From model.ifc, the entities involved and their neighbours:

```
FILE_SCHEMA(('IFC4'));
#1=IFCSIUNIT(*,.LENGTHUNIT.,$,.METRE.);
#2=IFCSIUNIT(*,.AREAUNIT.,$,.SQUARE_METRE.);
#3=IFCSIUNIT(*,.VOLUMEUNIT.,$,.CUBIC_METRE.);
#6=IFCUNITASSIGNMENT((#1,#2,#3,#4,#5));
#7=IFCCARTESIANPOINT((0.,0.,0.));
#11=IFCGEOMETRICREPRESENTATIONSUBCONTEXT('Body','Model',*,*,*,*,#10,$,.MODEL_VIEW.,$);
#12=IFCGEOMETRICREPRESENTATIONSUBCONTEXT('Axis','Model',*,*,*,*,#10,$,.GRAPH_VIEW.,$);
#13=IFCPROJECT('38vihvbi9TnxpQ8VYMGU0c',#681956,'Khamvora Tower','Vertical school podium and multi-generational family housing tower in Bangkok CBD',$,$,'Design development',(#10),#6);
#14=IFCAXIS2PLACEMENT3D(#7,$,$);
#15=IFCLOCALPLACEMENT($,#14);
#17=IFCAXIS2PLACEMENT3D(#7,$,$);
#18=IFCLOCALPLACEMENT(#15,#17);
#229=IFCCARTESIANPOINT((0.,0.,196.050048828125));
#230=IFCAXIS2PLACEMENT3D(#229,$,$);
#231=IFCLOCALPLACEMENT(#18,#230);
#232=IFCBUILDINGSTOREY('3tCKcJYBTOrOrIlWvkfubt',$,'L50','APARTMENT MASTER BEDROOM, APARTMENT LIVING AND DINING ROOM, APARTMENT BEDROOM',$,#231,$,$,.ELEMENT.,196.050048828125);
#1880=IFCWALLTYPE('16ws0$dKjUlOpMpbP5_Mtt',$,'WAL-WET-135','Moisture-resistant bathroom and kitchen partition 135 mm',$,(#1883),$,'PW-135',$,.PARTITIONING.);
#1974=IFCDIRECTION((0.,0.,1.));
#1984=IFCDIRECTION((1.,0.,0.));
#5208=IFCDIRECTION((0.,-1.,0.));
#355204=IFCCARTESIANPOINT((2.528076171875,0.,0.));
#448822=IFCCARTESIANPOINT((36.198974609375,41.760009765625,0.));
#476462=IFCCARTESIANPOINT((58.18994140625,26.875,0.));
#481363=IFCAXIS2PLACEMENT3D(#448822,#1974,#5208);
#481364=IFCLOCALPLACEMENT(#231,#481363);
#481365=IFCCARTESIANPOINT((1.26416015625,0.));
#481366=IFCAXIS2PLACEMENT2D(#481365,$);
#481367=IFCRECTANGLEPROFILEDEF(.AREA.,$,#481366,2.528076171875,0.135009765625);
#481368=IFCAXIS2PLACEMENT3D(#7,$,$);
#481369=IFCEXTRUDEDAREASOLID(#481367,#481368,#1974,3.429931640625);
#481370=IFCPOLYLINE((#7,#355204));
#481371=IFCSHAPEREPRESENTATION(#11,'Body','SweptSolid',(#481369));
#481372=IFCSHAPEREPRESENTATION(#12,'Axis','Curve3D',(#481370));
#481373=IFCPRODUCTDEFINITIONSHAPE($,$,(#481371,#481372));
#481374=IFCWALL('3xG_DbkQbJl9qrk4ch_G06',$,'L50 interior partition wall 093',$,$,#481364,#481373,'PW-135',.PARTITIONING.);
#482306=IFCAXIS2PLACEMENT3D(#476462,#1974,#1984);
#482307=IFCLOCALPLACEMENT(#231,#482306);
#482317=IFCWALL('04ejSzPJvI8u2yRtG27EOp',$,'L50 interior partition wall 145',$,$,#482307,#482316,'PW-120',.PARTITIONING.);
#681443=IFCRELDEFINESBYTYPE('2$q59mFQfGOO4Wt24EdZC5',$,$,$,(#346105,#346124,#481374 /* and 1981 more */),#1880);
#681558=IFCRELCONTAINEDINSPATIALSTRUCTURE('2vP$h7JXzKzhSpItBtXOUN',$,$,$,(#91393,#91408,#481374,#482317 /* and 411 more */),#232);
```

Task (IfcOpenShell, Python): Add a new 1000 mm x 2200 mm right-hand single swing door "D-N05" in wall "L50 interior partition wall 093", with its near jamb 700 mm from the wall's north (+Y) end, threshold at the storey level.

```python
import numpy as np
import ifcopenshell
import ifcopenshell.api.feature
import ifcopenshell.api.geometry
import ifcopenshell.api.root
import ifcopenshell.api.spatial
import ifcopenshell.geom
import ifcopenshell.util.element
import ifcopenshell.util.placement
import ifcopenshell.util.representation
import ifcopenshell.util.shape
import ifcopenshell.util.unit

model = ifcopenshell.open("model.ifc")
unit_scale = ifcopenshell.util.unit.calculate_unit_scale(model)
settings = ifcopenshell.geom.settings()


def volume(element):
    """Net volume in cubic metres, openings subtracted."""
    shape = ifcopenshell.geom.create_shape(settings, element)
    return ifcopenshell.util.shape.get_volume(shape.geometry)


wall = model.by_id(481374)
storey = ifcopenshell.util.element.get_container(wall, ifc_class="IfcBuildingStorey")
context = ifcopenshell.util.representation.get_context(model, "Model", "Body", "MODEL_VIEW")
before = volume(wall)

width, height, from_end, sill = 1, 2.2, 0.7, 0.0  # metres

# The wall runs along its own X axis, and the end named is its -X end.
wall_shape = ifcopenshell.geom.create_shape(settings, wall)
x, y, z = ifcopenshell.util.shape.get_vertices(wall_shape.geometry).T
start = x.min() + from_end
face, thickness = float(y.min()), float(y.max() - y.min())
wall_matrix = ifcopenshell.util.placement.get_local_placement(wall.ObjectPlacement)
level = ifcopenshell.util.placement.get_local_placement(storey.ObjectPlacement)[2, 3]


def in_wall(x, y):
    """Placement at x, y metres in the wall's axes, at sill height."""
    matrix = wall_matrix.copy()
    matrix[:, 3] = wall_matrix @ np.array([x / unit_scale, y / unit_scale, 0.0, 1.0])
    matrix[2, 3] = level + sill / unit_scale
    return matrix


# Opening: a box that overshoots both wall faces by 50 mm.
opening = ifcopenshell.api.root.create_entity(model, ifc_class="IfcOpeningElement", predefined_type="OPENING")
box = ifcopenshell.api.geometry.add_wall_representation(
    model, context=context, length=width, height=height, thickness=thickness + 0.1
)
ifcopenshell.api.geometry.assign_representation(model, product=opening, representation=box)
ifcopenshell.api.geometry.edit_object_placement(model, product=opening, matrix=in_wall(start, face - 0.05), is_si=False)
ifcopenshell.api.feature.add_feature(model, feature=opening, element=wall)

door = ifcopenshell.api.root.create_entity(model, ifc_class="IfcDoor", name="D-N05", predefined_type="DOOR")
door.OverallWidth, door.OverallHeight = width / unit_scale, height / unit_scale
door.OperationType = "SINGLE_SWING_RIGHT"
body = ifcopenshell.api.geometry.add_door_representation(
    model,
    context=context,
    overall_width=door.OverallWidth,
    overall_height=door.OverallHeight,
    operation_type="SINGLE_SWING_RIGHT",
    lining_properties={"LiningDepth": thickness / unit_scale, "ThresholdDepth": thickness / unit_scale},
)
ifcopenshell.api.geometry.assign_representation(model, product=door, representation=body)
ifcopenshell.api.spatial.assign_container(model, products=[door], relating_structure=storey)
ifcopenshell.api.feature.add_filling(model, opening=opening, element=door)

# The lining spans the wall, so the door starts at the wall face.
ifcopenshell.api.geometry.edit_object_placement(model, product=door, matrix=in_wall(start, face), is_si=False)

after = volume(wall)

print(f"wall volume {before:.3f} -> {after:.3f} m3")

model.write("model_edited.ifc")
```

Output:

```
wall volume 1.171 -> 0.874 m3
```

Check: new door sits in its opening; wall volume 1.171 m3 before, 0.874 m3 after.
